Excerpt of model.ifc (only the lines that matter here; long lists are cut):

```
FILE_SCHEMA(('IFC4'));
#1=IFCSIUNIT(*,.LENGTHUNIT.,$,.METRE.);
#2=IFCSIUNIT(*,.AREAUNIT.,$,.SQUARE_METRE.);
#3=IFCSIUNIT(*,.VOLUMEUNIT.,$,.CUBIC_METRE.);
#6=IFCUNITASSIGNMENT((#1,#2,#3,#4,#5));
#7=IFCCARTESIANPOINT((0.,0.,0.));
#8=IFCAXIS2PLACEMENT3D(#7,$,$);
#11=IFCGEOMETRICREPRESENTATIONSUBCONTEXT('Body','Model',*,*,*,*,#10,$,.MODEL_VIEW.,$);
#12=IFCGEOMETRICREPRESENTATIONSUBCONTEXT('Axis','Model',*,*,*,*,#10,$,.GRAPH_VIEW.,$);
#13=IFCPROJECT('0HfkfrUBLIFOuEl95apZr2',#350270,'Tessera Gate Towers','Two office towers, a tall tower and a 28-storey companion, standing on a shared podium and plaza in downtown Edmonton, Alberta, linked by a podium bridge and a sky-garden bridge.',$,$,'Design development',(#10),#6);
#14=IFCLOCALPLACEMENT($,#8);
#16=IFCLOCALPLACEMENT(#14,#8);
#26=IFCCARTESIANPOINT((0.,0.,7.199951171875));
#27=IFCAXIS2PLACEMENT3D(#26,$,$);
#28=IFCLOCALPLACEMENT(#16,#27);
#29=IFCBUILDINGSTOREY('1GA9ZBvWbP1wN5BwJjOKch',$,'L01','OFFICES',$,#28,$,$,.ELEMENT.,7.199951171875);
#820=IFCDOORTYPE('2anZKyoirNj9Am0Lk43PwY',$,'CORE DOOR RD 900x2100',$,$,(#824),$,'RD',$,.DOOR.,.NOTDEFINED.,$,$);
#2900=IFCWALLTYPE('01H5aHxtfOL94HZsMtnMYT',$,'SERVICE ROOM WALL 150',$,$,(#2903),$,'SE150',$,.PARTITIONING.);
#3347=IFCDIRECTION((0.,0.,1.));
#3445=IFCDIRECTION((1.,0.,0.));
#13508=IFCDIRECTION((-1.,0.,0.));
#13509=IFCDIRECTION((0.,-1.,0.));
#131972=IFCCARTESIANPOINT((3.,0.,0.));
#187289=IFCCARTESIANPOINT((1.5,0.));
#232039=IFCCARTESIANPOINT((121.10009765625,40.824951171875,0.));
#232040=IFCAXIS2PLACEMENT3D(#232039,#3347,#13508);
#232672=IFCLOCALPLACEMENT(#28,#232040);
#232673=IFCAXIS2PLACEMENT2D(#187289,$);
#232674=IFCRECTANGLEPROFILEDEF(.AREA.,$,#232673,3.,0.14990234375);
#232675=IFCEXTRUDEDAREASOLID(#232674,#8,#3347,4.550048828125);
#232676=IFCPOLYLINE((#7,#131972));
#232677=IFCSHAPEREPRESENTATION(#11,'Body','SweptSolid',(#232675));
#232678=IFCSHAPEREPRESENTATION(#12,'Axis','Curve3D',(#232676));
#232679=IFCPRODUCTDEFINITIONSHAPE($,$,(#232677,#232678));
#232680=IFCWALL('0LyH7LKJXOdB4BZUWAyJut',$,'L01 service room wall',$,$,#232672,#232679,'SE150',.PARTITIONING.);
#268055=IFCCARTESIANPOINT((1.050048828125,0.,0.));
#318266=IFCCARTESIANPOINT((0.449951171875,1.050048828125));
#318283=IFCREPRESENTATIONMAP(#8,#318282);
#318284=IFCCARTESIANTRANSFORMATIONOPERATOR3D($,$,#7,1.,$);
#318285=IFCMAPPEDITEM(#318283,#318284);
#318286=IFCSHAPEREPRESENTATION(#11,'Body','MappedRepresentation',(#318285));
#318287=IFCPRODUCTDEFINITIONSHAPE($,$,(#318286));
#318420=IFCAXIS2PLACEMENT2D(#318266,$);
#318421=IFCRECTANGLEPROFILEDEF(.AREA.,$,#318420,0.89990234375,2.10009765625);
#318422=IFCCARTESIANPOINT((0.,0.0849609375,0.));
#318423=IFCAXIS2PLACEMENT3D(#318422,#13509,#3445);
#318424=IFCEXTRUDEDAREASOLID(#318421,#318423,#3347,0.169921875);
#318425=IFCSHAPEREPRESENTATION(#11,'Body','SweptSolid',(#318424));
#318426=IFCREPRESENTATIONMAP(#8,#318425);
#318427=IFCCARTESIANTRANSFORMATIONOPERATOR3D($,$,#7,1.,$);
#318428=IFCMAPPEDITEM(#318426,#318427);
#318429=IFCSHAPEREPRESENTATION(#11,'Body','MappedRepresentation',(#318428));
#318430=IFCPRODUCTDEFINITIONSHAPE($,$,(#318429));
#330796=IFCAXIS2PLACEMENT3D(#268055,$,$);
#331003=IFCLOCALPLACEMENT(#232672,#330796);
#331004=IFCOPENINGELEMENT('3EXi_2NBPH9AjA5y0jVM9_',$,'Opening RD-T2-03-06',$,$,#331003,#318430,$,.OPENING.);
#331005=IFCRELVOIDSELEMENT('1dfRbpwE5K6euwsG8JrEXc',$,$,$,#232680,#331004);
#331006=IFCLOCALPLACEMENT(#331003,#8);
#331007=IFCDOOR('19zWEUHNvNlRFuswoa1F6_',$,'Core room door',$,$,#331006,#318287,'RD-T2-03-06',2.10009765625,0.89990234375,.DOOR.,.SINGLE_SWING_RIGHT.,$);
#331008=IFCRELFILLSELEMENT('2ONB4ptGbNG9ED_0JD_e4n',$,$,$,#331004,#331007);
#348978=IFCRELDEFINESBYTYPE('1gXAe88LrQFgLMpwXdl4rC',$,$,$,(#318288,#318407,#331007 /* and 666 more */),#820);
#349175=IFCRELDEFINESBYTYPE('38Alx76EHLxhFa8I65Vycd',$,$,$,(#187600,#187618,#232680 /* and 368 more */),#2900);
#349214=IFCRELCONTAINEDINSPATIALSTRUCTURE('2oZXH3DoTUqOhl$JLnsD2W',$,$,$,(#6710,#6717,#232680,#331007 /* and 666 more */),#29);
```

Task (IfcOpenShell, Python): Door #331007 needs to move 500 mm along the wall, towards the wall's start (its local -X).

```python
import ifcopenshell
import ifcopenshell.api.geometry
import ifcopenshell.util.placement
import ifcopenshell.util.unit

model = ifcopenshell.open("model.ifc")
unit_scale = ifcopenshell.util.unit.calculate_unit_scale(model)

door = model.by_guid("19zWEUHNvNlRFuswoa1F6_")
opening = door.FillsVoids[0].RelatingOpeningElement
wall = opening.VoidsElements[0].RelatingBuildingElement

wall_matrix = ifcopenshell.util.placement.get_local_placement(wall.ObjectPlacement)
shift = wall_matrix[:3, 0] * -0.5 / unit_scale
before = ifcopenshell.util.placement.get_local_placement(door.ObjectPlacement)[:3, 3].copy()

# The door is placed relative to its opening, so it follows when the opening moves.
matrix = ifcopenshell.util.placement.get_local_placement(opening.ObjectPlacement)
matrix[:3, 3] += shift
ifcopenshell.api.geometry.edit_object_placement(
    model, product=opening, matrix=matrix, is_si=False, should_transform_children=True
)

after = ifcopenshell.util.placement.get_local_placement(door.ObjectPlacement)[:3, 3]
print("door moved by", (after - before).round(3) + 0.0)

model.write("model_v2.ifc")
```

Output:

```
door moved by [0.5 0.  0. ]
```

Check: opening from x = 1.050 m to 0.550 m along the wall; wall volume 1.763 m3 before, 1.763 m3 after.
